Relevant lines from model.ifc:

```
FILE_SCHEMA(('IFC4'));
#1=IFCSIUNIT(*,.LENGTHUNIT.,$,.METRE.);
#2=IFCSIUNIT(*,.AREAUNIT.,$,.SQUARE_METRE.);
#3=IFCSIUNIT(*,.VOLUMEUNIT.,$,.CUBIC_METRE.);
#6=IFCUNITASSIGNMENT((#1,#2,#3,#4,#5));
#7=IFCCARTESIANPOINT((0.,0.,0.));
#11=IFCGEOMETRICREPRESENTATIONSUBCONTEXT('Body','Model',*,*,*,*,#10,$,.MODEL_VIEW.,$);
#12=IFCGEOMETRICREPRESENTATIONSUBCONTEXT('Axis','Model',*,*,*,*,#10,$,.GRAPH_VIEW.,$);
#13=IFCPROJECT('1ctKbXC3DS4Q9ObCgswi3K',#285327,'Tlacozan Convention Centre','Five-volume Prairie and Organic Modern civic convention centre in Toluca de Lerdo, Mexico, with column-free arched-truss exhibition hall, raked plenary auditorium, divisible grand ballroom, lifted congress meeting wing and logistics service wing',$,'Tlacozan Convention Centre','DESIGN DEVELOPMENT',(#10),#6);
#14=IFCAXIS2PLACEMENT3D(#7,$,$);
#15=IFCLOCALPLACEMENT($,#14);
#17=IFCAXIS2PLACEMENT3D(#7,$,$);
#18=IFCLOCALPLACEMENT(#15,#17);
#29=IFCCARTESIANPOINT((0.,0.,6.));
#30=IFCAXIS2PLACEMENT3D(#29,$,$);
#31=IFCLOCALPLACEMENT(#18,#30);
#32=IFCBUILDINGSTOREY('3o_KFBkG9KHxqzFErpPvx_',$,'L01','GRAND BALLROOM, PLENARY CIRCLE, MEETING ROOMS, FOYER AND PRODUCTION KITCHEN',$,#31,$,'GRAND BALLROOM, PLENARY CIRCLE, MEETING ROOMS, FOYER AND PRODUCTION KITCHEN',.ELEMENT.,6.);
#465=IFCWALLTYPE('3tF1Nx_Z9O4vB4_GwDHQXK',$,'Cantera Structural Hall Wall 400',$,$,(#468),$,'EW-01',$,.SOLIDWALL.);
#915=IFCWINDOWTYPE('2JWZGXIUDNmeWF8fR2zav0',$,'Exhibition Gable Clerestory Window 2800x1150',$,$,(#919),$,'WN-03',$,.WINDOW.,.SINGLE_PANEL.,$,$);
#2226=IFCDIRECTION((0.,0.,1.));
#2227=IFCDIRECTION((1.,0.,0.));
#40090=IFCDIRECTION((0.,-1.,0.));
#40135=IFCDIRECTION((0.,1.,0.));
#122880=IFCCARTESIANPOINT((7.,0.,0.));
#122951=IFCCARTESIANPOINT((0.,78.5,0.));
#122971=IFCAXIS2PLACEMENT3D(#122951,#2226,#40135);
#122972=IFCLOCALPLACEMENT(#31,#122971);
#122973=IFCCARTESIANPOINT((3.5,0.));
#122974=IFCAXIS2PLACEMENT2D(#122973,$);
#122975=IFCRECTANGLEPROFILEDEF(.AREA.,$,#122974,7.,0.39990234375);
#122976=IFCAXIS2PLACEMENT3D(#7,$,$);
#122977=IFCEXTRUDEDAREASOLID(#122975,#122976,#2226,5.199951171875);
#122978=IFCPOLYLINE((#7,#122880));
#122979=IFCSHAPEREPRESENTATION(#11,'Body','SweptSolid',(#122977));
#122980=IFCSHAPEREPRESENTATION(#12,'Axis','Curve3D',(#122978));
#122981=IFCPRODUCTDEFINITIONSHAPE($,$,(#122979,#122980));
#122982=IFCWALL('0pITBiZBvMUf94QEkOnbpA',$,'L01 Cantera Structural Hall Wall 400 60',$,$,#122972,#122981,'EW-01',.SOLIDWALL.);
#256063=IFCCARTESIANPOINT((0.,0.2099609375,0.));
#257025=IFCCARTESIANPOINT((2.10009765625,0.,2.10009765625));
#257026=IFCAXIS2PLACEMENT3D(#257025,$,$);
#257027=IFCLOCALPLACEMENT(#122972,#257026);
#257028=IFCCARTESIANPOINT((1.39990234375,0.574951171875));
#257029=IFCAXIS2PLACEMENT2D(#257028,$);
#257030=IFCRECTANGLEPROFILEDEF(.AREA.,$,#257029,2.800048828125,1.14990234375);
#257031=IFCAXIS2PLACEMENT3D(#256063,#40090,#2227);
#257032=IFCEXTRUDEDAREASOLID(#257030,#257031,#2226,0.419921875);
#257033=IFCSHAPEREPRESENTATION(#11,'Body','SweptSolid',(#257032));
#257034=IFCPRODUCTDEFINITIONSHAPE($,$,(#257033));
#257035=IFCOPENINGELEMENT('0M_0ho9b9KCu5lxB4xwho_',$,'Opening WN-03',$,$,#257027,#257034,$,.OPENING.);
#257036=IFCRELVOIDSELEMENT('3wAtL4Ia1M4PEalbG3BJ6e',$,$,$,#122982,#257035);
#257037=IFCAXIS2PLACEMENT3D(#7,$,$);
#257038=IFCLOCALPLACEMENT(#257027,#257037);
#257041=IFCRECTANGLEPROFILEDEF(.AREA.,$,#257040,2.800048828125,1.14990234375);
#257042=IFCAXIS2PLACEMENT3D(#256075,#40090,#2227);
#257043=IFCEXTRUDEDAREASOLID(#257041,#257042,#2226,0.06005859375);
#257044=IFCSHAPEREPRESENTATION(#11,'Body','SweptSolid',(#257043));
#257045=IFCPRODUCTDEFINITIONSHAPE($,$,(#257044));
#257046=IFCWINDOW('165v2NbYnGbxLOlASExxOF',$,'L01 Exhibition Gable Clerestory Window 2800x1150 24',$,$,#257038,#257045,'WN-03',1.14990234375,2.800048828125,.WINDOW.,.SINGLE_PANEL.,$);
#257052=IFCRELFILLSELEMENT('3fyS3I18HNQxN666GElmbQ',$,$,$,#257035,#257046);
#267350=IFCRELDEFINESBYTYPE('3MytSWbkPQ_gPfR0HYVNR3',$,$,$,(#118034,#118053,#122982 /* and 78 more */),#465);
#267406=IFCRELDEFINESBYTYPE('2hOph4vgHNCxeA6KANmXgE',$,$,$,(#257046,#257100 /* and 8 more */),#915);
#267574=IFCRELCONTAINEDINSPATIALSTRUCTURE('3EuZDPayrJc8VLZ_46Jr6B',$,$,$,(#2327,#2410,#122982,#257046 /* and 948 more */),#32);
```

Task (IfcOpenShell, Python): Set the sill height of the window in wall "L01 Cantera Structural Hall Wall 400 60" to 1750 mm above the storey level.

```python
import numpy as np
import ifcopenshell
import ifcopenshell.api.geometry
import ifcopenshell.geom
import ifcopenshell.util.element
import ifcopenshell.util.placement
import ifcopenshell.util.shape
import ifcopenshell.util.unit

model = ifcopenshell.open("model.ifc")
unit_scale = ifcopenshell.util.unit.calculate_unit_scale(model)

window = model.by_id(257046)
opening = window.FillsVoids[0].RelatingOpeningElement
storey = ifcopenshell.util.element.get_container(window, ifc_class="IfcBuildingStorey")
level = ifcopenshell.util.placement.get_local_placement(storey.ObjectPlacement)[2, 3]

# The opening's origin need not be at the sill, so measure its lowest point.
shape = ifcopenshell.geom.create_shape(ifcopenshell.geom.settings(), opening)
bottom = ifcopenshell.util.shape.get_shape_bottom_elevation(shape, shape.geometry) / unit_scale
dz = level + 1.75 / unit_scale - bottom

shift = np.array([0.0, 0.0, dz])
# The window is placed relative to its opening, so it follows when the opening moves.
matrix = ifcopenshell.util.placement.get_local_placement(opening.ObjectPlacement)
matrix[:3, 3] += shift
ifcopenshell.api.geometry.edit_object_placement(
    model, product=opening, matrix=matrix, is_si=False, should_transform_children=True
)

print(f"moved by {dz * unit_scale:+.3f} m")

model.write("model-out.ifc")
```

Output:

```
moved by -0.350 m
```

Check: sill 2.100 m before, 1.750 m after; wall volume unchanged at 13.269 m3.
